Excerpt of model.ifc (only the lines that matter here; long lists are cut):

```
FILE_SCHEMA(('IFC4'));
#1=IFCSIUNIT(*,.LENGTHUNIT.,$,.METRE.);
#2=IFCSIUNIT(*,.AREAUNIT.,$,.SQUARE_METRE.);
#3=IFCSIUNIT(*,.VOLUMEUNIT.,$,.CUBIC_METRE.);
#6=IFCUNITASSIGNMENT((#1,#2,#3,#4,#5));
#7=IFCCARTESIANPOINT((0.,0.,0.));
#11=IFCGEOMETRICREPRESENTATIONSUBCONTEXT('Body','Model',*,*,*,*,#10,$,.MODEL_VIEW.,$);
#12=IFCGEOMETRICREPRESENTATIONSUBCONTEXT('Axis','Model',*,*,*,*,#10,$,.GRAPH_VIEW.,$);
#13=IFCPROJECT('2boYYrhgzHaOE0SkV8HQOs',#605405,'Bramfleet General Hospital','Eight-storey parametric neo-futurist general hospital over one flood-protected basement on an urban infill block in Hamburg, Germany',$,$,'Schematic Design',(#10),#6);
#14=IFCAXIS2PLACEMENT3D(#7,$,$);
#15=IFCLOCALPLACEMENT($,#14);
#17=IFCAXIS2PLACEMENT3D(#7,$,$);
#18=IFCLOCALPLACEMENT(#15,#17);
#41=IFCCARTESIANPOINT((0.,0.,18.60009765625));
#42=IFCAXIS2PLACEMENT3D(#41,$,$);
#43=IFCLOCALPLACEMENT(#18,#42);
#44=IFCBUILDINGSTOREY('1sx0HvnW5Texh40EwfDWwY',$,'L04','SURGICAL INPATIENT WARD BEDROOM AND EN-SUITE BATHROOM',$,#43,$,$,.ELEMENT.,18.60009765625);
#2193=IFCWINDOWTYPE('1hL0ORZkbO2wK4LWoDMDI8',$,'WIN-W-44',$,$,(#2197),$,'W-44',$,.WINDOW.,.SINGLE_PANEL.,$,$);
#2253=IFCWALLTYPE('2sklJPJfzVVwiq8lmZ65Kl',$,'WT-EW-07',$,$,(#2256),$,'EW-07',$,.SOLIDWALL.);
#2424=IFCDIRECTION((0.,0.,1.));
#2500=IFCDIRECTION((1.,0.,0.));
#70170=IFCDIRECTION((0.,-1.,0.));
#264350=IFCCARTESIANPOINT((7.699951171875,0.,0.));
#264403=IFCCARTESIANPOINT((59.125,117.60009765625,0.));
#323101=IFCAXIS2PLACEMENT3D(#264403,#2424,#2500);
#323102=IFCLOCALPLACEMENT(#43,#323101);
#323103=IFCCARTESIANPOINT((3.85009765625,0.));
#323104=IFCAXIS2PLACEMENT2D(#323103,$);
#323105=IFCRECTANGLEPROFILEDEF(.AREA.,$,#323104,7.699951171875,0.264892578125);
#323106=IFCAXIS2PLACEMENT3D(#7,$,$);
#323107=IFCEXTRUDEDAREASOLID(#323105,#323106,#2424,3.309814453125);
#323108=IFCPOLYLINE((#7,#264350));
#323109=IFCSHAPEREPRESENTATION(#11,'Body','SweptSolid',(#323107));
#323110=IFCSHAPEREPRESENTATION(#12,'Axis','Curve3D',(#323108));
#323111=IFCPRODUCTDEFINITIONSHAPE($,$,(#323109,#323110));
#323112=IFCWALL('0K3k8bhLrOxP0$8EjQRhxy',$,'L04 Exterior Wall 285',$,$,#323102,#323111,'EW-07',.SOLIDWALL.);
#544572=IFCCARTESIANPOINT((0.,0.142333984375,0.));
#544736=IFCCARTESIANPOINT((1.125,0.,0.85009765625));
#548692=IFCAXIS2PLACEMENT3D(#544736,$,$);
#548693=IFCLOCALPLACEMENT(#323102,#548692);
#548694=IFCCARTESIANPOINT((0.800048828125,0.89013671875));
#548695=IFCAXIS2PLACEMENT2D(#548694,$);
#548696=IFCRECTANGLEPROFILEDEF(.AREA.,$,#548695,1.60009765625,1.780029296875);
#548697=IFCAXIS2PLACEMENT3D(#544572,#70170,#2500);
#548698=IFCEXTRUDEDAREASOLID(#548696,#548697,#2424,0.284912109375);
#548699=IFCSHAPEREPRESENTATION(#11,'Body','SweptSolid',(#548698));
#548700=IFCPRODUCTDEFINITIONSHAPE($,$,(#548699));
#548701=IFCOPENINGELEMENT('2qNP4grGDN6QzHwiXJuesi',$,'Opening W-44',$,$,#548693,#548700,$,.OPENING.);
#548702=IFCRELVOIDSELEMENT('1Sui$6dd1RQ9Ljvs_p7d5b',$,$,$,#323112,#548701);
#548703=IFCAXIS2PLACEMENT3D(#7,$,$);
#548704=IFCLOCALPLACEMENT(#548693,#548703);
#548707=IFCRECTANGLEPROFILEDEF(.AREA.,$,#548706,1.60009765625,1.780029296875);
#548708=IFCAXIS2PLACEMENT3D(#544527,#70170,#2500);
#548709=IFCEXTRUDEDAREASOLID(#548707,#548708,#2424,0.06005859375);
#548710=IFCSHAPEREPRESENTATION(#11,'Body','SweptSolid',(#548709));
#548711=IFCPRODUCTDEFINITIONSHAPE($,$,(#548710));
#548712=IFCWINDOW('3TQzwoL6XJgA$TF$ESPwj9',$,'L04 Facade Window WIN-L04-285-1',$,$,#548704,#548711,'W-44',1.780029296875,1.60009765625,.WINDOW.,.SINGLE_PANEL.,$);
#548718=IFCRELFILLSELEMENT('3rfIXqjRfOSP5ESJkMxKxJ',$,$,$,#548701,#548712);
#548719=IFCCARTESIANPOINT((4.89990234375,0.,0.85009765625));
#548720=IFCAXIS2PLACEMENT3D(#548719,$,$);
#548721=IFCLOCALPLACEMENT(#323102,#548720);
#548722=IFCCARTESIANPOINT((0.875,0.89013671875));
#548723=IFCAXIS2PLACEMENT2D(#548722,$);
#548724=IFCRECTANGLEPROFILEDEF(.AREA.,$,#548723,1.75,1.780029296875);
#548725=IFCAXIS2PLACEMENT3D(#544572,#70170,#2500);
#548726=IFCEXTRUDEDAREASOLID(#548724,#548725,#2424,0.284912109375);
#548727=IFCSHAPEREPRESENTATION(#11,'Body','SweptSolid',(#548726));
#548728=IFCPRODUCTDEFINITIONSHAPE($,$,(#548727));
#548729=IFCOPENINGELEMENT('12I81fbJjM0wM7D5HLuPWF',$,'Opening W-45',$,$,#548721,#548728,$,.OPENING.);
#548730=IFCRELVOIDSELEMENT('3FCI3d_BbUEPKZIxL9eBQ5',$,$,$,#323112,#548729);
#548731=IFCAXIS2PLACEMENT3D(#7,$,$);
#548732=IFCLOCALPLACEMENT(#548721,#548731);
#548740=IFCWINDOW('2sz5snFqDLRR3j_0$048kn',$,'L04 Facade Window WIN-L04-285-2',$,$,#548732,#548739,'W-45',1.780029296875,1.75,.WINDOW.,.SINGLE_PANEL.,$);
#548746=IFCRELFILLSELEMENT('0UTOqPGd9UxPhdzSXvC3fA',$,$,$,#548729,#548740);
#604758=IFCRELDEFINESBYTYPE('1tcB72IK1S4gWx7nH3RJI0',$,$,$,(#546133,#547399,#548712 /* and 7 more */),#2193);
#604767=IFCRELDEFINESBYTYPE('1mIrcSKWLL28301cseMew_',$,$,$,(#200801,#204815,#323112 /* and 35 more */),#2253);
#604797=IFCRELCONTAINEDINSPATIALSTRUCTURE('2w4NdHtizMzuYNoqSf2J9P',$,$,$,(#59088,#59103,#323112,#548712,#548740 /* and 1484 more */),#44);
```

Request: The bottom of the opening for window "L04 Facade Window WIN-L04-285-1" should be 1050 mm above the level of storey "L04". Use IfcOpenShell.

```python
import numpy as np
import ifcopenshell
import ifcopenshell.api.geometry
import ifcopenshell.geom
import ifcopenshell.util.element
import ifcopenshell.util.placement
import ifcopenshell.util.shape
import ifcopenshell.util.unit

model = ifcopenshell.open("model.ifc")
unit_scale = ifcopenshell.util.unit.calculate_unit_scale(model)

window = model.by_guid("3TQzwoL6XJgA$TF$ESPwj9")
opening = window.FillsVoids[0].RelatingOpeningElement
storey = ifcopenshell.util.element.get_container(window, ifc_class="IfcBuildingStorey")
level = ifcopenshell.util.placement.get_local_placement(storey.ObjectPlacement)[2, 3]

# The opening's origin need not be at the sill, so measure its lowest point.
shape = ifcopenshell.geom.create_shape(ifcopenshell.geom.settings(), opening)
bottom = ifcopenshell.util.shape.get_shape_bottom_elevation(shape, shape.geometry) / unit_scale
dz = level + 1.05 / unit_scale - bottom

shift = np.array([0.0, 0.0, dz])
# The window is placed relative to its opening, so it follows when the opening moves.
matrix = ifcopenshell.util.placement.get_local_placement(opening.ObjectPlacement)
matrix[:3, 3] += shift
ifcopenshell.api.geometry.edit_object_placement(
    model, product=opening, matrix=matrix, is_si=False, should_transform_children=True
)

print(f"moved by {dz * unit_scale:+.3f} m")

model.write("model_updated.ifc")
```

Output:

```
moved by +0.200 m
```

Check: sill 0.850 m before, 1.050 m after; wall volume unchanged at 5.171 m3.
